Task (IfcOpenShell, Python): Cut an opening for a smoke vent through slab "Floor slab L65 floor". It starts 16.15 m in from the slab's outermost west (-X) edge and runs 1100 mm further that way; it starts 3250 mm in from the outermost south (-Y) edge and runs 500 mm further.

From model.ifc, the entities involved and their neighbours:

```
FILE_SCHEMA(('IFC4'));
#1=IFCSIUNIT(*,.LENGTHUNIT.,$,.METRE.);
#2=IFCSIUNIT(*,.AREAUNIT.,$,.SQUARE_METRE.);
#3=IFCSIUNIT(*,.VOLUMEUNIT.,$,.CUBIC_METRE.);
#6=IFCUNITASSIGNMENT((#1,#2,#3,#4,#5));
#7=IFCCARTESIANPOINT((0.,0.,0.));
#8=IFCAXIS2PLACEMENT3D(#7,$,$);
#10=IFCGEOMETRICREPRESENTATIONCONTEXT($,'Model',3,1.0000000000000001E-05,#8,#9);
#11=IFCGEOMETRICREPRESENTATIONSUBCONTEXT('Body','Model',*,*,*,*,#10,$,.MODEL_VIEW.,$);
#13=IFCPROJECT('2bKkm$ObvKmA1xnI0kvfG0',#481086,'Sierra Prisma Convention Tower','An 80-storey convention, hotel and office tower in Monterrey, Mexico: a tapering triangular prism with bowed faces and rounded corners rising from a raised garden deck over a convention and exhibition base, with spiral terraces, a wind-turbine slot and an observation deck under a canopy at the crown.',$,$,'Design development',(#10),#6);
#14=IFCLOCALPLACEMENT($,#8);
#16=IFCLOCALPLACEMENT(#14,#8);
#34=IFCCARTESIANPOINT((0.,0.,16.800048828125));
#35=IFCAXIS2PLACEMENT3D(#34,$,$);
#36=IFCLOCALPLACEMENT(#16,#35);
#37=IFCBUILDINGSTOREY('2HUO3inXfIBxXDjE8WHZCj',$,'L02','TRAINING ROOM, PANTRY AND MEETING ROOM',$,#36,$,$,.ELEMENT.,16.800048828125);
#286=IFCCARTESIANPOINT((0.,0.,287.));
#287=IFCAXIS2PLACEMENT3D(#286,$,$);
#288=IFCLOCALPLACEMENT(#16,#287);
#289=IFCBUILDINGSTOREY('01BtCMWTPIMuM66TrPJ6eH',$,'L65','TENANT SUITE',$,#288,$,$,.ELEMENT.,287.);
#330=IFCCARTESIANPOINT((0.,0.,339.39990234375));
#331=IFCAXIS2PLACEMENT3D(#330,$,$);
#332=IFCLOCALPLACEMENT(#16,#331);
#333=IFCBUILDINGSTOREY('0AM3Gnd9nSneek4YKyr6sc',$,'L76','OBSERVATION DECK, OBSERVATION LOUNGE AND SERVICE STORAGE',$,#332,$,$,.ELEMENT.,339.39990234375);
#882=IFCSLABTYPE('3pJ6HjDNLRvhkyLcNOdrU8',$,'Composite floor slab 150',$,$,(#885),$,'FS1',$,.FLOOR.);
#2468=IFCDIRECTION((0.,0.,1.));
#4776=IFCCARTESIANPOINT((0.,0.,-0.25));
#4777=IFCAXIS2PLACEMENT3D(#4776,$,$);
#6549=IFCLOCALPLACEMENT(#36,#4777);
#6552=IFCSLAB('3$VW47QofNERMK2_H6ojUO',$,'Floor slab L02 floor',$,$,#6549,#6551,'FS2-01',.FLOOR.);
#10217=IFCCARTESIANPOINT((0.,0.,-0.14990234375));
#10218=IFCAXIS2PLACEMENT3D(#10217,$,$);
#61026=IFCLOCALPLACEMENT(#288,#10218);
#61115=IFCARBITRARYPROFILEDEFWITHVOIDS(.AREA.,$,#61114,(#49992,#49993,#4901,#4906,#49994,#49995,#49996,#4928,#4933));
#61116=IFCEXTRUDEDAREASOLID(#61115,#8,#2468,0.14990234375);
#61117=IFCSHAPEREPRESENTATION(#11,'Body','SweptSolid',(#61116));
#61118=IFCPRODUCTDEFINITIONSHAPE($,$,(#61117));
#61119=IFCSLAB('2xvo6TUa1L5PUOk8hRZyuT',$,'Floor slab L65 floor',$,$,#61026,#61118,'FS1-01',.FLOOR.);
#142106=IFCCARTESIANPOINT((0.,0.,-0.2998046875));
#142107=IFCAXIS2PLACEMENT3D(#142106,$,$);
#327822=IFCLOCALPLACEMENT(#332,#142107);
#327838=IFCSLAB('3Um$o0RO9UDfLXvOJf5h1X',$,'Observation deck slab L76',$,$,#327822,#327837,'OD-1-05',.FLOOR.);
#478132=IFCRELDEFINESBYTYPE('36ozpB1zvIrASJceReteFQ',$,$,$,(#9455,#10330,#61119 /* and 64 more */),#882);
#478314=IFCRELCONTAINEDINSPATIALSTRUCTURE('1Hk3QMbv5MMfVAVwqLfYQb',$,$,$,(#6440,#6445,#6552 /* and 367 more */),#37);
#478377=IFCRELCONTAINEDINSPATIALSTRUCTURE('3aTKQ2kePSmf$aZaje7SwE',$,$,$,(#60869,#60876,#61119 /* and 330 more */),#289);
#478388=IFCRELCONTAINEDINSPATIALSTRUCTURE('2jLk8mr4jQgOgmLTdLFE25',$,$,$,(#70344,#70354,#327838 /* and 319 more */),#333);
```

```python
import numpy as np
import ifcopenshell
import ifcopenshell.api.feature
import ifcopenshell.api.geometry
import ifcopenshell.api.root
import ifcopenshell.geom
import ifcopenshell.util.placement
import ifcopenshell.util.representation
import ifcopenshell.util.shape
import ifcopenshell.util.unit

model = ifcopenshell.open("model.ifc")
unit_scale = ifcopenshell.util.unit.calculate_unit_scale(model)
settings = ifcopenshell.geom.settings()


def volume(element):
    """Net volume in cubic metres, openings subtracted."""
    shape = ifcopenshell.geom.create_shape(settings, element)
    return ifcopenshell.util.shape.get_volume(shape.geometry)


slab = model.by_guid("2xvo6TUa1L5PUOk8hRZyuT")
before = volume(slab)

# Extent in the slab's own axes, in metres. The edges named are its -X and -Y sides.
slab_shape = ifcopenshell.geom.create_shape(settings, slab)
vertices = ifcopenshell.util.shape.get_vertices(slab_shape.geometry)
x_min, y_min, bottom = vertices.min(axis=0)
top = vertices[:, 2].max()

opening = ifcopenshell.api.root.create_entity(model, ifc_class="IfcOpeningElement", name="Smoke vent opening", predefined_type="OPENING")
context = ifcopenshell.util.representation.get_context(model, "Model", "Body", "MODEL_VIEW")
width, depth = 1.1, 0.5
outline = [(0.0, 0.0), (width, 0.0), (width, depth), (0.0, depth), (0.0, 0.0)]
# Overshoot both faces by 50 mm so the cut is clean.
shape = ifcopenshell.api.geometry.add_slab_representation(
    model, context=context, depth=top - bottom + 0.1, polyline=outline
)
ifcopenshell.api.geometry.assign_representation(model, product=opening, representation=shape)

matrix = ifcopenshell.util.placement.get_local_placement(slab.ObjectPlacement)
matrix[:, 3] = matrix @ np.append(np.array([x_min + 16.15, y_min + 3.25, bottom - 0.05]) / unit_scale, 1.0)
ifcopenshell.api.geometry.edit_object_placement(model, product=opening, matrix=matrix, is_si=False)
ifcopenshell.api.feature.add_feature(model, feature=opening, element=slab)

after = volume(slab)

print(f"slab volume {before:.3f} -> {after:.3f} m3")

model.write("model_rev.ifc")
```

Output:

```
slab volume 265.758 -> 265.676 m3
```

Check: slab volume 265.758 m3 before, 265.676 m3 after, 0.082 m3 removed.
